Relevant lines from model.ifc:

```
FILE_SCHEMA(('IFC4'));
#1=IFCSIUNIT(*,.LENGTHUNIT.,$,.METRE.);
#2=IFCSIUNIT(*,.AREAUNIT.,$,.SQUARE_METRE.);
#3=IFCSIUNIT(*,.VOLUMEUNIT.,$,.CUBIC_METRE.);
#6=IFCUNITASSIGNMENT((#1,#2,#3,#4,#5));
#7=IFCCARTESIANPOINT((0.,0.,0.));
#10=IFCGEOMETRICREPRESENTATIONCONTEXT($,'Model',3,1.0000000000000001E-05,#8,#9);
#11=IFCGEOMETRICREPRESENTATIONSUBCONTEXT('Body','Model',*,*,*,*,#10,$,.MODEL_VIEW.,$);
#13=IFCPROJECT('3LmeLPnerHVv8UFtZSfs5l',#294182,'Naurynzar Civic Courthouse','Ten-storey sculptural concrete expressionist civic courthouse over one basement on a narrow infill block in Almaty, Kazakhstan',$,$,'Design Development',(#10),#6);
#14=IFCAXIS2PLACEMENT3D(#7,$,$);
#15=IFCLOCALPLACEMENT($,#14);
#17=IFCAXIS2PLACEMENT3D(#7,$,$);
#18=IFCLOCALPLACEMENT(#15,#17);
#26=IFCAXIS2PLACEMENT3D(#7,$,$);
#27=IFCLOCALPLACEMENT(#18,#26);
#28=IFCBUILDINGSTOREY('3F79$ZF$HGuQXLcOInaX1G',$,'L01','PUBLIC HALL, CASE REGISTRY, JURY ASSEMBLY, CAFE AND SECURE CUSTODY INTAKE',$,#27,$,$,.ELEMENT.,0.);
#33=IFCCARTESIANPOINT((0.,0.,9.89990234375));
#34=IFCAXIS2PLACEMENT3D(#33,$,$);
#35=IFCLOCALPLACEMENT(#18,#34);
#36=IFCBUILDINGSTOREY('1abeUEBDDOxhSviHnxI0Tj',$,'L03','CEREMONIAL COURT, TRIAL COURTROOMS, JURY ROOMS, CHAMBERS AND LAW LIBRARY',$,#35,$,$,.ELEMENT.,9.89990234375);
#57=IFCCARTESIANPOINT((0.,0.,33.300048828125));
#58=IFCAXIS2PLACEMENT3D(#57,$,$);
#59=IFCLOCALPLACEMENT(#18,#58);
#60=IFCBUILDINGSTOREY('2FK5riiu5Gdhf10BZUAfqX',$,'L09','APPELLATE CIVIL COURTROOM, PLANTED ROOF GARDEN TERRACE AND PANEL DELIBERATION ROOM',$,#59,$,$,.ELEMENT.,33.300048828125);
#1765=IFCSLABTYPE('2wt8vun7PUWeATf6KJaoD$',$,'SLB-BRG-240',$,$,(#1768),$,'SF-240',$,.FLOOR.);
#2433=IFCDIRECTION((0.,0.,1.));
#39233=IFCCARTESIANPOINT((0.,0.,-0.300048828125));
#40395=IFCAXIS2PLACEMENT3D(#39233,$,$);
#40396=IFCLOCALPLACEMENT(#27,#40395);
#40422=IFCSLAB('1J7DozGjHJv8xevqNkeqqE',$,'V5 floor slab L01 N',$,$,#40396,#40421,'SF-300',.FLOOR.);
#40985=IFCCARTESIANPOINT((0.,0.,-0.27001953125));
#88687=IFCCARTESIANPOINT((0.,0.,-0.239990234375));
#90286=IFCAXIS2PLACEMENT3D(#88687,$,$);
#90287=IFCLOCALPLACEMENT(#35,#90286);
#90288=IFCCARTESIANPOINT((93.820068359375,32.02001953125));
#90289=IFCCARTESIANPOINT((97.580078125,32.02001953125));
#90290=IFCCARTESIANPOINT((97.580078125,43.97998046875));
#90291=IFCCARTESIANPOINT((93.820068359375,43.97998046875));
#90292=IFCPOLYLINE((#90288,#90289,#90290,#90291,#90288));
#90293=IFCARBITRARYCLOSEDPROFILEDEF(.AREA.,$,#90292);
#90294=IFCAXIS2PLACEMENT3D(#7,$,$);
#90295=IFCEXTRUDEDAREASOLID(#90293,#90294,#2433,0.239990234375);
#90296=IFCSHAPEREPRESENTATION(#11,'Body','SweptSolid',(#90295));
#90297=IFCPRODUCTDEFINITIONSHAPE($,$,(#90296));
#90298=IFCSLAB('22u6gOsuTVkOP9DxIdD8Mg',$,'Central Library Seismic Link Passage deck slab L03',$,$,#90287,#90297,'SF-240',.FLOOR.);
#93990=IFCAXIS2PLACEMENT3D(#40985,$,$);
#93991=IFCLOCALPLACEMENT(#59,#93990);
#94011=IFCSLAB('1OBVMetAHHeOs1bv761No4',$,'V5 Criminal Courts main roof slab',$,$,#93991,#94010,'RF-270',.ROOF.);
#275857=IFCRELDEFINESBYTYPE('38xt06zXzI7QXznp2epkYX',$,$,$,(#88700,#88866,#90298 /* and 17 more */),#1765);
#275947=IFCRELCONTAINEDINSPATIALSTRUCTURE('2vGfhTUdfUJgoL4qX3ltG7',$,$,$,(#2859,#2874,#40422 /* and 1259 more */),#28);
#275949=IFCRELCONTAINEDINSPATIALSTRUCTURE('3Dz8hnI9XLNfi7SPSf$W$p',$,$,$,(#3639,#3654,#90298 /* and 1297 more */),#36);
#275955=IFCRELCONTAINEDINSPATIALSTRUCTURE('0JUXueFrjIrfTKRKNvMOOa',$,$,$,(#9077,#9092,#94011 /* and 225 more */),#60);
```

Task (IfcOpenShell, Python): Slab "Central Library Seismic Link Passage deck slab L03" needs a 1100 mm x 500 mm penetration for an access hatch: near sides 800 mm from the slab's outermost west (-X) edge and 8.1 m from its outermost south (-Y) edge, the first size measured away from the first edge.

```python
import numpy as np
import ifcopenshell
import ifcopenshell.api.feature
import ifcopenshell.api.geometry
import ifcopenshell.api.root
import ifcopenshell.geom
import ifcopenshell.util.placement
import ifcopenshell.util.representation
import ifcopenshell.util.shape
import ifcopenshell.util.unit

model = ifcopenshell.open("model.ifc")
unit_scale = ifcopenshell.util.unit.calculate_unit_scale(model)
settings = ifcopenshell.geom.settings()


def volume(element):
    """Net volume in cubic metres, openings subtracted."""
    shape = ifcopenshell.geom.create_shape(settings, element)
    return ifcopenshell.util.shape.get_volume(shape.geometry)


slab = model.by_id(90298)
before = volume(slab)

# Extent in the slab's own axes, in metres. The edges named are its -X and -Y sides.
slab_shape = ifcopenshell.geom.create_shape(settings, slab)
vertices = ifcopenshell.util.shape.get_vertices(slab_shape.geometry)
x_min, y_min, bottom = vertices.min(axis=0)
top = vertices[:, 2].max()

opening = ifcopenshell.api.root.create_entity(model, ifc_class="IfcOpeningElement", name="Access hatch opening", predefined_type="OPENING")
context = ifcopenshell.util.representation.get_context(model, "Model", "Body", "MODEL_VIEW")
width, depth = 1.1, 0.5
outline = [(0.0, 0.0), (width, 0.0), (width, depth), (0.0, depth), (0.0, 0.0)]
# Overshoot both faces by 50 mm so the cut is clean.
shape = ifcopenshell.api.geometry.add_slab_representation(
    model, context=context, depth=top - bottom + 0.1, polyline=outline
)
ifcopenshell.api.geometry.assign_representation(model, product=opening, representation=shape)

matrix = ifcopenshell.util.placement.get_local_placement(slab.ObjectPlacement)
matrix[:, 3] = matrix @ np.append(np.array([x_min + 0.8, y_min + 8.1, bottom - 0.05]) / unit_scale, 1.0)
ifcopenshell.api.geometry.edit_object_placement(model, product=opening, matrix=matrix, is_si=False)
ifcopenshell.api.feature.add_feature(model, feature=opening, element=slab)

after = volume(slab)

print(f"slab volume {before:.3f} -> {after:.3f} m3")

model.write("model-out.ifc")
```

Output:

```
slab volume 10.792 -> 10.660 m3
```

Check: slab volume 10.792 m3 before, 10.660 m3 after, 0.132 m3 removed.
